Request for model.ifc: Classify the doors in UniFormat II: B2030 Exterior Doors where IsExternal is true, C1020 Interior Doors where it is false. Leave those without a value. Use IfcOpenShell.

First a look at what the model holds.

```python
import ifcopenshell
import ifcopenshell.util.element

model = ifcopenshell.open("model.ifc")
print(model.schema)
print("classifications:", [c.Name for c in model.by_type("IfcClassification")])
values = [ifcopenshell.util.element.get_pset(e, "Pset_DoorCommon", "IsExternal") for e in model.by_type("IfcDoor")]
for value in (True, False, None):
    print("IsExternal", value, values.count(value))
```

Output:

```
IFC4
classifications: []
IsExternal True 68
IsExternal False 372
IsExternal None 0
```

```python
import ifcopenshell
import ifcopenshell.api.classification
import ifcopenshell.util.element

model = ifcopenshell.open("model.ifc")

system = ifcopenshell.api.classification.add_classification(model, classification="UniFormat II")

doors = model.by_type("IfcDoor")
external = {e: ifcopenshell.util.element.get_pset(e, "Pset_DoorCommon", "IsExternal") for e in doors}
for flag, code, name in ((True, "B2030", "Exterior Doors"), (False, "C1020", "Interior Doors")):
    products = [e for e in doors if external[e] is flag]
    ifcopenshell.api.classification.add_reference(
        model, products=products, classification=system, identification=code, name=name
    )
    print(code, len(products))

model.write("model_updated.ifc")
```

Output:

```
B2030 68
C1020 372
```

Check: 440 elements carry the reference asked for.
